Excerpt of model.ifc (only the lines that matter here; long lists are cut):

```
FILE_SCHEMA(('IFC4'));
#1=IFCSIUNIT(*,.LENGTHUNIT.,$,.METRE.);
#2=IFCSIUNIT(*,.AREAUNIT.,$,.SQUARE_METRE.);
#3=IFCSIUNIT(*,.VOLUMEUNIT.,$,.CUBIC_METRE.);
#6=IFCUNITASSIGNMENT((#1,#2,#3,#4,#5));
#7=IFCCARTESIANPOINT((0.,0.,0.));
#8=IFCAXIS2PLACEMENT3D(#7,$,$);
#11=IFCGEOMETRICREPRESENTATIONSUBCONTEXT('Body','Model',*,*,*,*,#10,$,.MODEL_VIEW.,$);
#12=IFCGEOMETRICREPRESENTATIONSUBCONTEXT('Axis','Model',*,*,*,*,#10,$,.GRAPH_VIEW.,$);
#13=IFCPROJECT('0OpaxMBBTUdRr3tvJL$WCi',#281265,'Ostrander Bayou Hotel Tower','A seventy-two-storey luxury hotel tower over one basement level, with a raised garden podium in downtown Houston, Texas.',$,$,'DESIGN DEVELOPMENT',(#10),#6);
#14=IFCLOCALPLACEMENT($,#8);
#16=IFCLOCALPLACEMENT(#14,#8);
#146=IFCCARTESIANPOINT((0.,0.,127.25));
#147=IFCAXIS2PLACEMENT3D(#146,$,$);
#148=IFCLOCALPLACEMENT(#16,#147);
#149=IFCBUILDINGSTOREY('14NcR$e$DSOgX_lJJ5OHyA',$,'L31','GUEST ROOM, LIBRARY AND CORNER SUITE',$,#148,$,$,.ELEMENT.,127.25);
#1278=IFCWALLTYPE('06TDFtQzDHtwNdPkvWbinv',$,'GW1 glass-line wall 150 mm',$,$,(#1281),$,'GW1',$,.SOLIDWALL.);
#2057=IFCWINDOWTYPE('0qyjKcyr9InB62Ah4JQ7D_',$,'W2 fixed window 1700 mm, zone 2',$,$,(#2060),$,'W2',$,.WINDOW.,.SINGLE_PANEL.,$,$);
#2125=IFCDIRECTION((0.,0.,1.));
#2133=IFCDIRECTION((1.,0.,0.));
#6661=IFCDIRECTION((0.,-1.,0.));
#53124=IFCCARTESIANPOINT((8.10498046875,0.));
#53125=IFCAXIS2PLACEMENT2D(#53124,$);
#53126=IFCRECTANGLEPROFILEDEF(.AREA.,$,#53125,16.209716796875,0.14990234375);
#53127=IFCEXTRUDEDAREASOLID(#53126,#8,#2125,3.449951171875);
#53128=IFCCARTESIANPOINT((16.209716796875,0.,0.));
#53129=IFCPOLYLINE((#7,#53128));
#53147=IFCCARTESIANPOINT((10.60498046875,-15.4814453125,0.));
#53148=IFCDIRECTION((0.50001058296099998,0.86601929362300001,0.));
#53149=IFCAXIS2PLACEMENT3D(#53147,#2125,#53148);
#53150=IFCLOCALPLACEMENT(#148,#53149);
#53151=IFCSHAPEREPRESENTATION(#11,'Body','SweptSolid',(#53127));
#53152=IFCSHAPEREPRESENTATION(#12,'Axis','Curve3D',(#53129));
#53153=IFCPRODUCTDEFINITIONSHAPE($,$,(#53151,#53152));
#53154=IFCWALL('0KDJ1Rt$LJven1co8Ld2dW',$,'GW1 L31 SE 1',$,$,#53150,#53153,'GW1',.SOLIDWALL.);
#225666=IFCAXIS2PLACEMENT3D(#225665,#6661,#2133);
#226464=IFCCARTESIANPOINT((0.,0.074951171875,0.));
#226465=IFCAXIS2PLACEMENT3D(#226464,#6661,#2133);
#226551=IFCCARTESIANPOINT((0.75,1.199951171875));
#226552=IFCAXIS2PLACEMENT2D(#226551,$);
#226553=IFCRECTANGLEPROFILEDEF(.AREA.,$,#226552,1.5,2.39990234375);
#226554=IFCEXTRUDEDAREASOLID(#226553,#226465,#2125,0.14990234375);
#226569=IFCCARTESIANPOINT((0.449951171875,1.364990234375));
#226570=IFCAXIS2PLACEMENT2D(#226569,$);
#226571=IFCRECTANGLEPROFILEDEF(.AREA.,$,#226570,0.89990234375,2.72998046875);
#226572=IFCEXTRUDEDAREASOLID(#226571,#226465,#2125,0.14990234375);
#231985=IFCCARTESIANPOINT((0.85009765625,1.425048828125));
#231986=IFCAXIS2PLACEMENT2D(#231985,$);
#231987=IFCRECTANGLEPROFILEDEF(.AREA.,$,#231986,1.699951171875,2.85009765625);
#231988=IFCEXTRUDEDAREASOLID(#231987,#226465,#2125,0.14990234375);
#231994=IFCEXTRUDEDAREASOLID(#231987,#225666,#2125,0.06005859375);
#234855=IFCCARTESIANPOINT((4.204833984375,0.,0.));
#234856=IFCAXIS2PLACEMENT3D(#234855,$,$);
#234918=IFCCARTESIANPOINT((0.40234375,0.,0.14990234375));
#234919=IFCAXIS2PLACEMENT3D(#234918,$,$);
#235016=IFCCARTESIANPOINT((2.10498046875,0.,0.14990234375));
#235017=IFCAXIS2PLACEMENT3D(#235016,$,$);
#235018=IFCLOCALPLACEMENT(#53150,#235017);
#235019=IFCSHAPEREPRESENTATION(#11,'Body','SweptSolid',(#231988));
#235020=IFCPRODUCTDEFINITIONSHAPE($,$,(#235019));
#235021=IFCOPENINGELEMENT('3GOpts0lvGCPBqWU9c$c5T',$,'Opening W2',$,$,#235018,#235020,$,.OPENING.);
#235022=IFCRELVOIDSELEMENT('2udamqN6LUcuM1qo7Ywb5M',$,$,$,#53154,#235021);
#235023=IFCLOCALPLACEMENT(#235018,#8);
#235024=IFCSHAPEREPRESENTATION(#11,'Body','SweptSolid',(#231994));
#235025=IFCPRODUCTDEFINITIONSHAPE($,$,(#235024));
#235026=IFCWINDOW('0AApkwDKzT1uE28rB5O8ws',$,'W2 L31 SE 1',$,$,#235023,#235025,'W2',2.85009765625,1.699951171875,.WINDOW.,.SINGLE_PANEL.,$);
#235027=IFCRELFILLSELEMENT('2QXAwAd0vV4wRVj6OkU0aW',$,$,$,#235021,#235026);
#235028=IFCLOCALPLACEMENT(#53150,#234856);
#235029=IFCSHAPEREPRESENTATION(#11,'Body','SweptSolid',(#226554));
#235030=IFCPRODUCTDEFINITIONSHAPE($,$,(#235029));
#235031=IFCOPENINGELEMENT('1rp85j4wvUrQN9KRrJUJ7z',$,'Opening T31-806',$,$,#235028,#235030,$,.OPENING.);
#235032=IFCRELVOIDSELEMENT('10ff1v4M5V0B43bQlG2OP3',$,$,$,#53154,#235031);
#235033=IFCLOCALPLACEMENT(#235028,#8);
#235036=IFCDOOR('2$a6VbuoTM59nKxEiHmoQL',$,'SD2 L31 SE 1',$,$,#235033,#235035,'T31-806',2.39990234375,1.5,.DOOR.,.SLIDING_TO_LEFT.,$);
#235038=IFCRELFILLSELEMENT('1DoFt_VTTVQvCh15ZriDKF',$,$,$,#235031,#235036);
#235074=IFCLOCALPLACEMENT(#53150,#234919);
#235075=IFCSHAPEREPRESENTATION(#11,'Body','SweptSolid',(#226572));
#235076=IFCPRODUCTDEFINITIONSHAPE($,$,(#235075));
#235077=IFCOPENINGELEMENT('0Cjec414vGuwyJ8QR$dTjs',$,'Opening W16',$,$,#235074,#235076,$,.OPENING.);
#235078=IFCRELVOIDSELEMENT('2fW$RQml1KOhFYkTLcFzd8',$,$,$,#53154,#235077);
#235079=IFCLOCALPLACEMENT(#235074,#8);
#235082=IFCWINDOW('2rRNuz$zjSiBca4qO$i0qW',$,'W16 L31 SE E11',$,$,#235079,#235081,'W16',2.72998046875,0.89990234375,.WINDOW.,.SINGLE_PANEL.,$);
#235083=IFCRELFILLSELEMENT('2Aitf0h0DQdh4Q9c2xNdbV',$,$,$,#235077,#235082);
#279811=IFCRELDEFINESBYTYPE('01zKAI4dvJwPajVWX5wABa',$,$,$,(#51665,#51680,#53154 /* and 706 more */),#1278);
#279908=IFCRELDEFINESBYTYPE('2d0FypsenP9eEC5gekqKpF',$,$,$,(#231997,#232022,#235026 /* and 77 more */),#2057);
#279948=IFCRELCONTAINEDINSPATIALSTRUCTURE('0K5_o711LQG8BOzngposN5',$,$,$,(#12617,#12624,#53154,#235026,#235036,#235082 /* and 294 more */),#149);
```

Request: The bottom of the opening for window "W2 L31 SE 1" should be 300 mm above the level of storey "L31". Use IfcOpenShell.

```python
import numpy as np
import ifcopenshell
import ifcopenshell.api.geometry
import ifcopenshell.geom
import ifcopenshell.util.element
import ifcopenshell.util.placement
import ifcopenshell.util.shape
import ifcopenshell.util.unit

model = ifcopenshell.open("model.ifc")
unit_scale = ifcopenshell.util.unit.calculate_unit_scale(model)

window = model.by_guid("0AApkwDKzT1uE28rB5O8ws")
opening = window.FillsVoids[0].RelatingOpeningElement
storey = ifcopenshell.util.element.get_container(window, ifc_class="IfcBuildingStorey")
level = ifcopenshell.util.placement.get_local_placement(storey.ObjectPlacement)[2, 3]

# The opening's origin need not be at the sill, so measure its lowest point.
shape = ifcopenshell.geom.create_shape(ifcopenshell.geom.settings(), opening)
bottom = ifcopenshell.util.shape.get_shape_bottom_elevation(shape, shape.geometry) / unit_scale
dz = level + 0.3 / unit_scale - bottom

shift = np.array([0.0, 0.0, dz])
# The window is placed relative to its opening, so it follows when the opening moves.
matrix = ifcopenshell.util.placement.get_local_placement(opening.ObjectPlacement)
matrix[:3, 3] += shift
ifcopenshell.api.geometry.edit_object_placement(
    model, product=opening, matrix=matrix, is_si=False, should_transform_children=True
)

print(f"moved by {dz * unit_scale:+.3f} m")

model.write("model_rev.ifc")
```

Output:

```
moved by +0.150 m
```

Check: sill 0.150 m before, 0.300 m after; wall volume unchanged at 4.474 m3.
